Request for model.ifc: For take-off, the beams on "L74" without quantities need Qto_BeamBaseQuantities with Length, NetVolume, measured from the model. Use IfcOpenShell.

First a look at what the model holds.

```python
import ifcopenshell
import ifcopenshell.util.element
import ifcopenshell.util.unit

model = ifcopenshell.open("model.ifc")
print(model.schema)
for unit_type in ("LENGTHUNIT", "AREAUNIT", "VOLUMEUNIT"):
    print(unit_type, ifcopenshell.util.unit.calculate_unit_scale(model, unit_type))
storey = next(s for s in model.by_type("IfcBuildingStorey") if s.Name == "L74")
beams = [e for e in ifcopenshell.util.element.get_decomposition(storey) if e.is_a("IfcBeam")]
for e in sorted(beams, key=lambda e: e.id()):
    print(e.id(), e.is_a(), e.Name, list(ifcopenshell.util.element.get_psets(e, qtos_only=True)), sep=" | ")
```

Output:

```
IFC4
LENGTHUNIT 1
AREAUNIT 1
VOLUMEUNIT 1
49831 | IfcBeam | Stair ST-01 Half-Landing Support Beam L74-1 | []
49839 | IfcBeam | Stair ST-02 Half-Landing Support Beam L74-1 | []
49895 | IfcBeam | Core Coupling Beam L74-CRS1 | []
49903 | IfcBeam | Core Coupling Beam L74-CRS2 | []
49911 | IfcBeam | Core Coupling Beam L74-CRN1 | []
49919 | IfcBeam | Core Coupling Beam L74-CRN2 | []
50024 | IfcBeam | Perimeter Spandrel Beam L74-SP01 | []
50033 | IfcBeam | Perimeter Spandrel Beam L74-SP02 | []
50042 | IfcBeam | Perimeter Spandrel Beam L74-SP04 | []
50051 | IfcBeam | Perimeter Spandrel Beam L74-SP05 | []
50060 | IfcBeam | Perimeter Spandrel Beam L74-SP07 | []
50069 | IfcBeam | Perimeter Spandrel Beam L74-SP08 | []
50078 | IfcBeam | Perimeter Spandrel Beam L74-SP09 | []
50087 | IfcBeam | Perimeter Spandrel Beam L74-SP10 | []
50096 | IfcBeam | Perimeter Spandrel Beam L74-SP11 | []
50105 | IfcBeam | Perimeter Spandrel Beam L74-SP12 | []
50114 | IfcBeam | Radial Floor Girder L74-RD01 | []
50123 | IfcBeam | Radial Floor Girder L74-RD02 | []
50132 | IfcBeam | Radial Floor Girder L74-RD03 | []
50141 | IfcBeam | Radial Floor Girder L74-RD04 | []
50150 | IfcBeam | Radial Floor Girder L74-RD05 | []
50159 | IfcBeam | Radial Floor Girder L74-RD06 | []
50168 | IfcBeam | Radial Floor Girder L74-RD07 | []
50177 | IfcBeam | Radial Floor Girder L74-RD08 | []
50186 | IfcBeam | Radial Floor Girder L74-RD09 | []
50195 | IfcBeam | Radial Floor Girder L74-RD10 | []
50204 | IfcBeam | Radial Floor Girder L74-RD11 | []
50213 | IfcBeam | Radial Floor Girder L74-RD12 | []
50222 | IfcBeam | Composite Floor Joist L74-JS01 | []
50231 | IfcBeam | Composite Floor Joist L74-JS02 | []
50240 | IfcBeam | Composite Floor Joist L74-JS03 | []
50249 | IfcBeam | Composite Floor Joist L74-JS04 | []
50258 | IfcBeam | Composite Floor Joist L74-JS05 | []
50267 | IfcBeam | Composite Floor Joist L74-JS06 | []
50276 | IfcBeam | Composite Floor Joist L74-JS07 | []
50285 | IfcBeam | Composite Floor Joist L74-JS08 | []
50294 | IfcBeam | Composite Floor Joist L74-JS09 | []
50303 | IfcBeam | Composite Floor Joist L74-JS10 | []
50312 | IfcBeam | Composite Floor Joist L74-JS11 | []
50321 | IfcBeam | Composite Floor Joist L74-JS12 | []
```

```python
import ifcopenshell
import ifcopenshell.api.pset
import ifcopenshell.geom
import ifcopenshell.util.element
import ifcopenshell.util.shape
import ifcopenshell.util.unit

model = ifcopenshell.open("model.ifc")
unit_scale = ifcopenshell.util.unit.calculate_unit_scale(model)
volume_scale = ifcopenshell.util.unit.calculate_unit_scale(model, "VOLUMEUNIT")
settings = ifcopenshell.geom.settings()

storey = next(s for s in model.by_type("IfcBuildingStorey") if s.Name == "L74")
beams = [e for e in ifcopenshell.util.element.get_decomposition(storey) if e.is_a("IfcBeam")]

for e in sorted(beams, key=lambda e: e.id()):
    if ifcopenshell.util.element.get_psets(e, qtos_only=True, should_inherit=False):
        continue
    # Geometry comes back in metres, in the element's own axes.
    shape = ifcopenshell.geom.create_shape(settings, e)
    values = {
        "Length": ifcopenshell.util.shape.get_max_xyz(shape.geometry) / unit_scale,
        "NetVolume": ifcopenshell.util.shape.get_volume(shape.geometry) / volume_scale,
    }
    qto = ifcopenshell.api.pset.add_qto(model, product=e, name="Qto_BeamBaseQuantities")
    ifcopenshell.api.pset.edit_qto(model, qto=qto, properties=values)
    print(e.id(), {k: round(v, 3) for k, v in values.items()})

model.write("model_v2.ifc")
```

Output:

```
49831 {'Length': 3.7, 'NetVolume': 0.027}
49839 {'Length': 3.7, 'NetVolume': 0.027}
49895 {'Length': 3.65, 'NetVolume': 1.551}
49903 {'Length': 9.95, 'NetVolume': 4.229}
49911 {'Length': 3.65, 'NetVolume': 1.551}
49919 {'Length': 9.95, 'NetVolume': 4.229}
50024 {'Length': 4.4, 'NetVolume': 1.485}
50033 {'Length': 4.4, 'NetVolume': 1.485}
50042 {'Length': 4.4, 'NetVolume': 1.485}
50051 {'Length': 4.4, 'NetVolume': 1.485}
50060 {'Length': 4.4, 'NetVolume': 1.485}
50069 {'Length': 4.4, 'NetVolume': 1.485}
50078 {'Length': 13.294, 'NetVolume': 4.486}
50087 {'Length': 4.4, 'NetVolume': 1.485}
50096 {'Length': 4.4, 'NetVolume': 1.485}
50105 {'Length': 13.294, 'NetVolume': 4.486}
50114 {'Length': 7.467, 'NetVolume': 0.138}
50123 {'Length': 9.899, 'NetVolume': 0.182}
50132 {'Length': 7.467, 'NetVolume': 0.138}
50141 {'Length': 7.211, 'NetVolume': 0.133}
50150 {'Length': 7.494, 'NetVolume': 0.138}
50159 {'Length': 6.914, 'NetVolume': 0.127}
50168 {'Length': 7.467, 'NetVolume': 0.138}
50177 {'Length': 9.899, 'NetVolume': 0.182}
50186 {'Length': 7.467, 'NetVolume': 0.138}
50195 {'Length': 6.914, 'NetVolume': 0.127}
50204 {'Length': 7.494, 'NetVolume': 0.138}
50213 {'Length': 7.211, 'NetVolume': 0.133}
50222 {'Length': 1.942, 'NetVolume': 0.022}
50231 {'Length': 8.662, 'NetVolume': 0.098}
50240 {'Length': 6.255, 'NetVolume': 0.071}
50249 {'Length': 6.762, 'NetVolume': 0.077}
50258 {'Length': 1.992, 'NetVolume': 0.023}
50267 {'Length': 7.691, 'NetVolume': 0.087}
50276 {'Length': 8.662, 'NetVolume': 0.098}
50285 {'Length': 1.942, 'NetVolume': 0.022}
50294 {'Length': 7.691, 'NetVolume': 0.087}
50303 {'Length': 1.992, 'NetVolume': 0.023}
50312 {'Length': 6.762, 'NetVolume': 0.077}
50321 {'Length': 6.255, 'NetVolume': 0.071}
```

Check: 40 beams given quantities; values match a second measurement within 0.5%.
